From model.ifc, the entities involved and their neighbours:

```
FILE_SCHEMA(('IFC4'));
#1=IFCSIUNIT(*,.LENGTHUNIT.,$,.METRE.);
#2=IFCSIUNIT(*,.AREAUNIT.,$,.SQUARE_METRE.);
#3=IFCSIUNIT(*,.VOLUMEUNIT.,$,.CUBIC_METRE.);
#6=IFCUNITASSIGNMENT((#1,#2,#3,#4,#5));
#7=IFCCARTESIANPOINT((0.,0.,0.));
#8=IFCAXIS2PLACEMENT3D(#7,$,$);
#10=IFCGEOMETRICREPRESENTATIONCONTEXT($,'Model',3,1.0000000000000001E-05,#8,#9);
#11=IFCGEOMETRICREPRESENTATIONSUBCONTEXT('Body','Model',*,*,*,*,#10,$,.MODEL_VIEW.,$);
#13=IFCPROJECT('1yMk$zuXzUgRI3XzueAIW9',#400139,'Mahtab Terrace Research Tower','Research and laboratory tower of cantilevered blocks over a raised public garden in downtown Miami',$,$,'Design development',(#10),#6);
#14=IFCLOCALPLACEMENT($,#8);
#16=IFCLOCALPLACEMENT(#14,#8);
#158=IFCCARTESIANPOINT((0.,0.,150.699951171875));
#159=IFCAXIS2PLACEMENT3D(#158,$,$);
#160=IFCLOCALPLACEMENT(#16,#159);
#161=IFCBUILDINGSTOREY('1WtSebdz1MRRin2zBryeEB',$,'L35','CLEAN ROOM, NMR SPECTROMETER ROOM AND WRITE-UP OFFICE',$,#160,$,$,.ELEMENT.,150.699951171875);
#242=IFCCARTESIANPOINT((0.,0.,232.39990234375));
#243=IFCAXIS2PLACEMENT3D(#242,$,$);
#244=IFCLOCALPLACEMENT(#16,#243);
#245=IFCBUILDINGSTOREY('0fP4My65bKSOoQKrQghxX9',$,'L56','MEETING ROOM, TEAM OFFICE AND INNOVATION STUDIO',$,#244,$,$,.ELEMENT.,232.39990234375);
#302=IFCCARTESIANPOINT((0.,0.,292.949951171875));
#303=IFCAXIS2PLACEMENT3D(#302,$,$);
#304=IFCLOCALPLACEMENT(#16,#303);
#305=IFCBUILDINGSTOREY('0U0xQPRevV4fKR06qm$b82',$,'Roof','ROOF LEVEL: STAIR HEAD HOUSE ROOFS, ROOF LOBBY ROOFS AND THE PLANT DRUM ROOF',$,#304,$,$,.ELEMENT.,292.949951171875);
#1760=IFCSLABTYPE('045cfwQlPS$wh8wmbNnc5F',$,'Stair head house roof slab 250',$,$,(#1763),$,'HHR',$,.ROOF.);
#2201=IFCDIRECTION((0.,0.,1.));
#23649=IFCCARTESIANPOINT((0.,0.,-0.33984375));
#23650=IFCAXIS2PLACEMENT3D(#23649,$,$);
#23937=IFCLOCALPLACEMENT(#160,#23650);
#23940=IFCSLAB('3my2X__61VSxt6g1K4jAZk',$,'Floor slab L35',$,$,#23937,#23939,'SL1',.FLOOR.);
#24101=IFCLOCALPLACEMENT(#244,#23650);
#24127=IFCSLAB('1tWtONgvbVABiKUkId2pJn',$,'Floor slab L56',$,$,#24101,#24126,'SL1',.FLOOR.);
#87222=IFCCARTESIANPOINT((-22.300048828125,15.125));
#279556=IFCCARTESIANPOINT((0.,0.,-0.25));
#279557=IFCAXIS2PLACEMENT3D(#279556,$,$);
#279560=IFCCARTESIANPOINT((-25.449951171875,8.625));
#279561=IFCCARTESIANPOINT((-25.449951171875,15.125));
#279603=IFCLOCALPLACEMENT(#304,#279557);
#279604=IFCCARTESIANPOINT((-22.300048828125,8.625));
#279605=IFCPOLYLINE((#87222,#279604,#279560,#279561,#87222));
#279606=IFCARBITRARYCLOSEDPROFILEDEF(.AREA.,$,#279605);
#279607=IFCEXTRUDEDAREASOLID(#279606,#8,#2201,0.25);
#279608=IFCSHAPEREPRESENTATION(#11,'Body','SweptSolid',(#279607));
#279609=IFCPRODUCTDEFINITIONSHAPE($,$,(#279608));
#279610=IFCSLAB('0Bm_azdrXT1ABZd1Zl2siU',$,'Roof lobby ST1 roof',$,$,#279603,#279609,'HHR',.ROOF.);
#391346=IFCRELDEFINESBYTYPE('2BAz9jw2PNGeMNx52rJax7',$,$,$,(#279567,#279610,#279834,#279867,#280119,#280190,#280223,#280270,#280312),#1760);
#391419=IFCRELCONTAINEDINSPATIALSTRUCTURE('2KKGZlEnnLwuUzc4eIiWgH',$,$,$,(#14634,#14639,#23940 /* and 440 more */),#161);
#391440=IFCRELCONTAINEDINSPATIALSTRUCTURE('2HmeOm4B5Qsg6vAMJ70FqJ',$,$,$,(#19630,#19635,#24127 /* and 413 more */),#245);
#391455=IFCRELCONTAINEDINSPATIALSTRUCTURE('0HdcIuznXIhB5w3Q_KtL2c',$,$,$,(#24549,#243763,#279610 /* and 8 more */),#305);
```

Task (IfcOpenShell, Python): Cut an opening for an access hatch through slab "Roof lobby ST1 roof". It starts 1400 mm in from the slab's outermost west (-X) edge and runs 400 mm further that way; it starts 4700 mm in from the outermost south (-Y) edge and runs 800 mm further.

```python
import numpy as np
import ifcopenshell
import ifcopenshell.api.feature
import ifcopenshell.api.geometry
import ifcopenshell.api.root
import ifcopenshell.geom
import ifcopenshell.util.placement
import ifcopenshell.util.representation
import ifcopenshell.util.shape
import ifcopenshell.util.unit

model = ifcopenshell.open("model.ifc")
unit_scale = ifcopenshell.util.unit.calculate_unit_scale(model)
settings = ifcopenshell.geom.settings()


def volume(element):
    """Net volume in cubic metres, openings subtracted."""
    shape = ifcopenshell.geom.create_shape(settings, element)
    return ifcopenshell.util.shape.get_volume(shape.geometry)


slab = model.by_guid("0Bm_azdrXT1ABZd1Zl2siU")
before = volume(slab)

# Extent in the slab's own axes, in metres. The edges named are its -X and -Y sides.
slab_shape = ifcopenshell.geom.create_shape(settings, slab)
vertices = ifcopenshell.util.shape.get_vertices(slab_shape.geometry)
x_min, y_min, bottom = vertices.min(axis=0)
top = vertices[:, 2].max()

opening = ifcopenshell.api.root.create_entity(model, ifc_class="IfcOpeningElement", name="Access hatch opening", predefined_type="OPENING")
context = ifcopenshell.util.representation.get_context(model, "Model", "Body", "MODEL_VIEW")
width, depth = 0.4, 0.8
outline = [(0.0, 0.0), (width, 0.0), (width, depth), (0.0, depth), (0.0, 0.0)]
# Overshoot both faces by 50 mm so the cut is clean.
shape = ifcopenshell.api.geometry.add_slab_representation(
    model, context=context, depth=top - bottom + 0.1, polyline=outline
)
ifcopenshell.api.geometry.assign_representation(model, product=opening, representation=shape)

matrix = ifcopenshell.util.placement.get_local_placement(slab.ObjectPlacement)
matrix[:, 3] = matrix @ np.append(np.array([x_min + 1.4, y_min + 4.7, bottom - 0.05]) / unit_scale, 1.0)
ifcopenshell.api.geometry.edit_object_placement(model, product=opening, matrix=matrix, is_si=False)
ifcopenshell.api.feature.add_feature(model, feature=opening, element=slab)

after = volume(slab)

print(f"slab volume {before:.3f} -> {after:.3f} m3")

model.write("model-out.ifc")
```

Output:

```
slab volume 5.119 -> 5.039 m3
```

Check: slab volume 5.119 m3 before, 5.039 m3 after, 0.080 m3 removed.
